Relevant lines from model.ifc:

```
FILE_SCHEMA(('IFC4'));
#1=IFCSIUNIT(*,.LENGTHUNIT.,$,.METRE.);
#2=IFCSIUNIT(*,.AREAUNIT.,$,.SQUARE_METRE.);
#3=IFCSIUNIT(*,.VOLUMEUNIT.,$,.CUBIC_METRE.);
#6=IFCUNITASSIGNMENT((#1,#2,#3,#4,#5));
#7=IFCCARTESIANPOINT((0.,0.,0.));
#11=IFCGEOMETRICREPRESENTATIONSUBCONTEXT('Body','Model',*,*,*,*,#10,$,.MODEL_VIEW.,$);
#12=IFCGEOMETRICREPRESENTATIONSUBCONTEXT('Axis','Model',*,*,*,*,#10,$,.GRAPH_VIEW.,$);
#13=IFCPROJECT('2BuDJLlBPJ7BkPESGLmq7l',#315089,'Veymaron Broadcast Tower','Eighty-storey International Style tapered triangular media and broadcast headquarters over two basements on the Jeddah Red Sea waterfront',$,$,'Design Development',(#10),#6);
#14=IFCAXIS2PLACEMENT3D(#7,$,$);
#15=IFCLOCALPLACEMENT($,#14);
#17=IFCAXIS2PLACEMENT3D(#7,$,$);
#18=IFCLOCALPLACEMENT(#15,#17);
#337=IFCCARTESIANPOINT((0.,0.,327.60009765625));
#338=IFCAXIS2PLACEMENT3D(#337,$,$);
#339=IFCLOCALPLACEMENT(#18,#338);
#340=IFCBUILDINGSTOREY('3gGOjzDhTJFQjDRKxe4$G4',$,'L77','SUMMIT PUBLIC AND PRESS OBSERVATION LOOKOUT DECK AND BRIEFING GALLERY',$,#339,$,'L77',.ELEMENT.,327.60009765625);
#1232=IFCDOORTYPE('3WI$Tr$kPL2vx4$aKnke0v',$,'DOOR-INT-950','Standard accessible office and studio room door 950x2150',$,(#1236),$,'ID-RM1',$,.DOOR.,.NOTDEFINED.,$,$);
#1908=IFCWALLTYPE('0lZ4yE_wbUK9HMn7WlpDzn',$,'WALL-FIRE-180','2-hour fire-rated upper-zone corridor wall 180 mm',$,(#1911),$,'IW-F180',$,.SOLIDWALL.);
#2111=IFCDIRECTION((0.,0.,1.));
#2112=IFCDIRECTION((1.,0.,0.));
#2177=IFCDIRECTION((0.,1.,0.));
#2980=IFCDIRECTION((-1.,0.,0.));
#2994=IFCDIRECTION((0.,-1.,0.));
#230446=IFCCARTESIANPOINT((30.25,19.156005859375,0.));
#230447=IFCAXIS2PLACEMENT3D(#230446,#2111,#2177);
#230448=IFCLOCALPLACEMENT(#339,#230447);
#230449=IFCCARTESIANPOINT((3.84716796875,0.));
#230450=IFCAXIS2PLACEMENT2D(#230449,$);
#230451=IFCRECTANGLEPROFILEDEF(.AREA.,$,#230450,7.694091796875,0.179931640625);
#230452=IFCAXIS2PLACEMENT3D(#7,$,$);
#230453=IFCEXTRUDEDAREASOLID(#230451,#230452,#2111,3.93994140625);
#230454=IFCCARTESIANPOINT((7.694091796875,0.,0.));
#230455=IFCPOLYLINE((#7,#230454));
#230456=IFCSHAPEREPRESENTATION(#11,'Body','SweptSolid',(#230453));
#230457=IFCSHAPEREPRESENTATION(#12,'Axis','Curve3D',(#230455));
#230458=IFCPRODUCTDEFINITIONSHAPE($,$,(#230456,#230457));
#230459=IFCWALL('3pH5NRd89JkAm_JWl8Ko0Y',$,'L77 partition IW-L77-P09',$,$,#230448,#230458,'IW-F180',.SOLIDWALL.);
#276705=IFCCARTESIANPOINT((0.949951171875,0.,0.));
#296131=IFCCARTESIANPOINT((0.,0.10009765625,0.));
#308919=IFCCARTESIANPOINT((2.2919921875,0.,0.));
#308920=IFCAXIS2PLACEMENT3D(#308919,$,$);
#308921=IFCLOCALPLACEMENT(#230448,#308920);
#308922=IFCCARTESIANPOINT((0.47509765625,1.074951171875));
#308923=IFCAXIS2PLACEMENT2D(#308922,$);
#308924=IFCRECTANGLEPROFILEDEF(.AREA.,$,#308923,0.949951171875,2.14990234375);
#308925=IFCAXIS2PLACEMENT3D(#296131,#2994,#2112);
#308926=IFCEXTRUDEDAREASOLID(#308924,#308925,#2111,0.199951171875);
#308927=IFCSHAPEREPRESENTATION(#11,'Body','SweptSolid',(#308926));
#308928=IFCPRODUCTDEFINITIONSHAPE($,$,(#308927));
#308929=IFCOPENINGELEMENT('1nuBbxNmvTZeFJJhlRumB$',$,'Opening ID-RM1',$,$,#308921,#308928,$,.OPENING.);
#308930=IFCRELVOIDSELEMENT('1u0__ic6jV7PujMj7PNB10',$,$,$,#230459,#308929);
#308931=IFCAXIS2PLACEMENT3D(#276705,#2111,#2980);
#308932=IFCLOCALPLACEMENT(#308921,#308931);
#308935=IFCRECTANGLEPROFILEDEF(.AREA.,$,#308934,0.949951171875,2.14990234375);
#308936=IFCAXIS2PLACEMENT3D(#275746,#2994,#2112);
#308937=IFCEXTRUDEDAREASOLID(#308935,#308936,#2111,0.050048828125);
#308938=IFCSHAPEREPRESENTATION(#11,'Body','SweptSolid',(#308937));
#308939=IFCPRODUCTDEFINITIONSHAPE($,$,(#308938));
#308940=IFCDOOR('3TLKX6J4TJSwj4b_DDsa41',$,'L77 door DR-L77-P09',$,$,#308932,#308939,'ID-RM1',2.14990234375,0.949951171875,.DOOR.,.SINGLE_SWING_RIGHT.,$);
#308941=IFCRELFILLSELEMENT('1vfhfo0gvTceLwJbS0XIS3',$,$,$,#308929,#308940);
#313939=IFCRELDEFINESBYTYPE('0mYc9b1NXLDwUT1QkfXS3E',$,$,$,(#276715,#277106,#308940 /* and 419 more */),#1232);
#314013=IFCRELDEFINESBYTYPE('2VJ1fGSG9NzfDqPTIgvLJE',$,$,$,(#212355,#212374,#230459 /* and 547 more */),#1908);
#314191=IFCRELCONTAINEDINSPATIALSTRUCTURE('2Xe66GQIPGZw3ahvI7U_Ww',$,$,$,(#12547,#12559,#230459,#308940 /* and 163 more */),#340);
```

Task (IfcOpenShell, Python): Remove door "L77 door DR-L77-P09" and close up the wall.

```python
import ifcopenshell
import ifcopenshell.api.feature
import ifcopenshell.api.root
import ifcopenshell.geom
import ifcopenshell.util.shape

model = ifcopenshell.open("model.ifc")
settings = ifcopenshell.geom.settings()


def volume(element):
    """Net volume in cubic metres, openings subtracted."""
    shape = ifcopenshell.geom.create_shape(settings, element)
    return ifcopenshell.util.shape.get_volume(shape.geometry)


door = model.by_guid("3TLKX6J4TJSwj4b_DDsa41")
opening = door.FillsVoids[0].RelatingOpeningElement
wall = opening.VoidsElements[0].RelatingBuildingElement
before = volume(wall)

ifcopenshell.api.root.remove_product(model, product=door)
ifcopenshell.api.feature.remove_feature(model, feature=opening)

after = volume(wall)

print(f"wall volume {before:.3f} -> {after:.3f} m3")

model.write("model_rev.ifc")
```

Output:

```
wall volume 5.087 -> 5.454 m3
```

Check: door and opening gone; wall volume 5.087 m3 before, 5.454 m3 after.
